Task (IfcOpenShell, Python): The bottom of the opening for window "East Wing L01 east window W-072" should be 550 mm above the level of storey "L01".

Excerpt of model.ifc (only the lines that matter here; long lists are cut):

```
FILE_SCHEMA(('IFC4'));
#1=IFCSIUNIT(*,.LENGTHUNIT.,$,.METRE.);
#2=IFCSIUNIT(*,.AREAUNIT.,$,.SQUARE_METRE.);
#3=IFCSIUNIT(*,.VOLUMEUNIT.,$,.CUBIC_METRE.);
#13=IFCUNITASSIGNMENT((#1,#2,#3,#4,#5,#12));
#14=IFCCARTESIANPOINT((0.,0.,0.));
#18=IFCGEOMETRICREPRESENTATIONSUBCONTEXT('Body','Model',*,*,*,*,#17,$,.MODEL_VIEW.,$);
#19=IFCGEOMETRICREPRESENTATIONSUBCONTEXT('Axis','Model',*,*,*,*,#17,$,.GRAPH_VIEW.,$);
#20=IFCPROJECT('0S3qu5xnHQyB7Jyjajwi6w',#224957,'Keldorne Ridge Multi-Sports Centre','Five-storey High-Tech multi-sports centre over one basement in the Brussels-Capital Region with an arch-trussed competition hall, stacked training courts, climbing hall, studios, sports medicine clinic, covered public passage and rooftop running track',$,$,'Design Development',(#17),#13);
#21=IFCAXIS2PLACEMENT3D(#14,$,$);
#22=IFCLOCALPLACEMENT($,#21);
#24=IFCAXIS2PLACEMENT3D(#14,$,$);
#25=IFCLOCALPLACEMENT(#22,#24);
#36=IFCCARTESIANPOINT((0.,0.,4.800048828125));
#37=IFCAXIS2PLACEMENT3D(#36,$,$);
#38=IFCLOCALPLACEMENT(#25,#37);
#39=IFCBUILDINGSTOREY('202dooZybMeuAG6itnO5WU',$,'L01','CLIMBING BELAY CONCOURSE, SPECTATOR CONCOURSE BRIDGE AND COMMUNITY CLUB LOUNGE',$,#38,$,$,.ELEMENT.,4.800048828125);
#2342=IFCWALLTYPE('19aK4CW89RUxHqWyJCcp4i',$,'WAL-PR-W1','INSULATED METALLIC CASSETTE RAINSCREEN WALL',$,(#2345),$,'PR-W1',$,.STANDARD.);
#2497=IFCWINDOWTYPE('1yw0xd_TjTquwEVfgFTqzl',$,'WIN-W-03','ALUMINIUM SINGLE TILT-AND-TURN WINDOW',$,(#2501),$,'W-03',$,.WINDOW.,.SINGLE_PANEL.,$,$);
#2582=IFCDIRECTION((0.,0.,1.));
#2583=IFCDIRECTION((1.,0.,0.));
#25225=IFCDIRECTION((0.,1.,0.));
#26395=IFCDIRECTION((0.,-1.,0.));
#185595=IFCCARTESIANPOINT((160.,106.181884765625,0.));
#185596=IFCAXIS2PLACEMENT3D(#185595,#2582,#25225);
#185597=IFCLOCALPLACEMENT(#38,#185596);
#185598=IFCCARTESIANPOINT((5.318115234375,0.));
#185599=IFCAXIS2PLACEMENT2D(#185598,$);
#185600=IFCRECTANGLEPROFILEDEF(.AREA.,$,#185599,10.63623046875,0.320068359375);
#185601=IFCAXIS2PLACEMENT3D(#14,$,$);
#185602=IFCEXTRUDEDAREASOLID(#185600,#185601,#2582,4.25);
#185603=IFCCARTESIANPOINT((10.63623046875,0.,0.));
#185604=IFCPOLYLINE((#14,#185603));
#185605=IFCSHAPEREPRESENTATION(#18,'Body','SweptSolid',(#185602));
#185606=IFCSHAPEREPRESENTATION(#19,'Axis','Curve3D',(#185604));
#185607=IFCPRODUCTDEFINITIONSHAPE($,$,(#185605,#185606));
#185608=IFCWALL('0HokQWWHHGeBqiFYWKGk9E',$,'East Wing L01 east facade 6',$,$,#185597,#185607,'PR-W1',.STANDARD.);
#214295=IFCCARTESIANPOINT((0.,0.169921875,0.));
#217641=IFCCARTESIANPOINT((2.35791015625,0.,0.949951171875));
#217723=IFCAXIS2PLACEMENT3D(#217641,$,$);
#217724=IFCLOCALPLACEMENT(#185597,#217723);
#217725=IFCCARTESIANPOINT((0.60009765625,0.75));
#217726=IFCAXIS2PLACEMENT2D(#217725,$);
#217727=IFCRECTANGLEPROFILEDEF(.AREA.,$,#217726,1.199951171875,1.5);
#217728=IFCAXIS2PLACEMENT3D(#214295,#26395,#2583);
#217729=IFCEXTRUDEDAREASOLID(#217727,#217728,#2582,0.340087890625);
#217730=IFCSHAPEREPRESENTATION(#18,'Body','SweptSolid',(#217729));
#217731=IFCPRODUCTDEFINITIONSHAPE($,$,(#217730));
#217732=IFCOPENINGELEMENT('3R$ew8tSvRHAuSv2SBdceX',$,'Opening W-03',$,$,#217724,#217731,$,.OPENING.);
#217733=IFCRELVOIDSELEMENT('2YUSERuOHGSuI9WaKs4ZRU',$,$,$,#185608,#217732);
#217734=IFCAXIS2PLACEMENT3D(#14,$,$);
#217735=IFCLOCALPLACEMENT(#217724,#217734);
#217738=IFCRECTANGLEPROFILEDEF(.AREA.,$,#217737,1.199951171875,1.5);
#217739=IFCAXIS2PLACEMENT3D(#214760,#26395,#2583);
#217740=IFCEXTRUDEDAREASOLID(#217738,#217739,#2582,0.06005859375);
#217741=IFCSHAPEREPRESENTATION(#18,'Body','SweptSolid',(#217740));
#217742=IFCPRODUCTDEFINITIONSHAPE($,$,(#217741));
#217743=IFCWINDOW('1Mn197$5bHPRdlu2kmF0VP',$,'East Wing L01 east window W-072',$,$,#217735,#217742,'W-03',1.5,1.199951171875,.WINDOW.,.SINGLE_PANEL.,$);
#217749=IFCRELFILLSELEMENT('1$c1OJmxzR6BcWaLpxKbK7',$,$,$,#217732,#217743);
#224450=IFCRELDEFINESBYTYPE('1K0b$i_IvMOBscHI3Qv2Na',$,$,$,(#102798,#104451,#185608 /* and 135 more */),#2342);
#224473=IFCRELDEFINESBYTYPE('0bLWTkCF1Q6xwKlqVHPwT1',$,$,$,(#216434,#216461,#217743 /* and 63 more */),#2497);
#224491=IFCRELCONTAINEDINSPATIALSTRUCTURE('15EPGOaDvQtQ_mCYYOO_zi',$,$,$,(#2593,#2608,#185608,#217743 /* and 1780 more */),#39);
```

```python
import numpy as np
import ifcopenshell
import ifcopenshell.api.geometry
import ifcopenshell.geom
import ifcopenshell.util.element
import ifcopenshell.util.placement
import ifcopenshell.util.shape
import ifcopenshell.util.unit

model = ifcopenshell.open("model.ifc")
unit_scale = ifcopenshell.util.unit.calculate_unit_scale(model)

window = model.by_guid("1Mn197$5bHPRdlu2kmF0VP")
opening = window.FillsVoids[0].RelatingOpeningElement
storey = ifcopenshell.util.element.get_container(window, ifc_class="IfcBuildingStorey")
level = ifcopenshell.util.placement.get_local_placement(storey.ObjectPlacement)[2, 3]

# The opening's origin need not be at the sill, so measure its lowest point.
shape = ifcopenshell.geom.create_shape(ifcopenshell.geom.settings(), opening)
bottom = ifcopenshell.util.shape.get_shape_bottom_elevation(shape, shape.geometry) / unit_scale
dz = level + 0.55 - bottom

shift = np.array([0.0, 0.0, dz])
# The window is placed relative to its opening, so it follows when the opening moves.
matrix = ifcopenshell.util.placement.get_local_placement(opening.ObjectPlacement)
matrix[:3, 3] += shift
ifcopenshell.api.geometry.edit_object_placement(
    model, product=opening, matrix=matrix, is_si=False, should_transform_children=True
)

print(f"moved by {dz * unit_scale:+.3f} m")

model.write("model-out.ifc")
```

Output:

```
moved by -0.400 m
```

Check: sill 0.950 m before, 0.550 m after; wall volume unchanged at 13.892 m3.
